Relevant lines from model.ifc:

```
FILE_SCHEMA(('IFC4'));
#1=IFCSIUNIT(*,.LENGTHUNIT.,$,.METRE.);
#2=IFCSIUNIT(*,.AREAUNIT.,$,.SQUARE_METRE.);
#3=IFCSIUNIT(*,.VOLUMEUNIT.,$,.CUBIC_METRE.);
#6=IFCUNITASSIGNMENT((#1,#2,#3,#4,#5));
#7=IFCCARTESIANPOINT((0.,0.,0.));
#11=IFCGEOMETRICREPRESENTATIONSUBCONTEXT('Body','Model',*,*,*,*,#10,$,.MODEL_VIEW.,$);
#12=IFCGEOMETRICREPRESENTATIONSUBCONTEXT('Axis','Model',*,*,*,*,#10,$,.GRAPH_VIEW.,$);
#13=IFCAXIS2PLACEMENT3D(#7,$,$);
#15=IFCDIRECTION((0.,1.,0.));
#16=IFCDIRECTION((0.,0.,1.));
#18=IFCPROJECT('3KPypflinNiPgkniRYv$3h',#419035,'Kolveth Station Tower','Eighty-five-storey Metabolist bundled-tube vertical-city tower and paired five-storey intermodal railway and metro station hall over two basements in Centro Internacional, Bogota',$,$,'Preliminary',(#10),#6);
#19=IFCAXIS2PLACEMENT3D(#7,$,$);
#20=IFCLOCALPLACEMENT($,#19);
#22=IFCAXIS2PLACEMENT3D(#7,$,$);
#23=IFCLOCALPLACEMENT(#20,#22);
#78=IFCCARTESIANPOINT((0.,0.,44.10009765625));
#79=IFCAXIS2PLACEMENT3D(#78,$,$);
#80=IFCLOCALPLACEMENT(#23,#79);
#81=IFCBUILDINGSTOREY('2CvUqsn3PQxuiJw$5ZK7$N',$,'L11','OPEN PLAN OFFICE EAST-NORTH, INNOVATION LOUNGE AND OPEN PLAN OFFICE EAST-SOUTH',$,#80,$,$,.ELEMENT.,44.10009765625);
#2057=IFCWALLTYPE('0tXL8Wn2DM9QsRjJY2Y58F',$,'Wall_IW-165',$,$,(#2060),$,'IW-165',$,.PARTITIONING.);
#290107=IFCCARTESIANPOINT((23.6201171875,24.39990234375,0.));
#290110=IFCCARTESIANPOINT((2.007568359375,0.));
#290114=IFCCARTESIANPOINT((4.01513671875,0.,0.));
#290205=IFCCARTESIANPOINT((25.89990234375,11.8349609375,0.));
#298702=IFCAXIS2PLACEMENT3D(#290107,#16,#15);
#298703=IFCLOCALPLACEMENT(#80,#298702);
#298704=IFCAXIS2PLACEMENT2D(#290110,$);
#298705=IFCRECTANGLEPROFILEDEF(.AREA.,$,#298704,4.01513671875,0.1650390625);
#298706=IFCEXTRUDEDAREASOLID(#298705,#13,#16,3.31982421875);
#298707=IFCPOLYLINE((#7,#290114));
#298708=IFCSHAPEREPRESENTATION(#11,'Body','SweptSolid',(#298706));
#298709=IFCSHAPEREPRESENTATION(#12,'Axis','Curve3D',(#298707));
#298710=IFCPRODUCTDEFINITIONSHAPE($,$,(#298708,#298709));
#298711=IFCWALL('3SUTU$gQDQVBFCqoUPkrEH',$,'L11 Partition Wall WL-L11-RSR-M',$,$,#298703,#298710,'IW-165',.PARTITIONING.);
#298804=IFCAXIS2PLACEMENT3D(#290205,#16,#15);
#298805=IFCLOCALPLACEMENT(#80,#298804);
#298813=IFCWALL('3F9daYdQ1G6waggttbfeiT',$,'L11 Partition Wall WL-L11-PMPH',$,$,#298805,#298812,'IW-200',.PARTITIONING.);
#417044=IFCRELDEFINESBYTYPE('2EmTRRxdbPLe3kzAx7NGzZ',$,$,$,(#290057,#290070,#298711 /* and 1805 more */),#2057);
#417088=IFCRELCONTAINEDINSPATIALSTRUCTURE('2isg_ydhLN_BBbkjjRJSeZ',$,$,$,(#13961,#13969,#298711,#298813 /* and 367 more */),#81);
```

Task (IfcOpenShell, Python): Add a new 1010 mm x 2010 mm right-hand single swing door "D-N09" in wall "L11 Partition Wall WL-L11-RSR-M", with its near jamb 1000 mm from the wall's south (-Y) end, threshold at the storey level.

```python
import numpy as np
import ifcopenshell
import ifcopenshell.api.feature
import ifcopenshell.api.geometry
import ifcopenshell.api.root
import ifcopenshell.api.spatial
import ifcopenshell.geom
import ifcopenshell.util.element
import ifcopenshell.util.placement
import ifcopenshell.util.representation
import ifcopenshell.util.shape
import ifcopenshell.util.unit

model = ifcopenshell.open("model.ifc")
unit_scale = ifcopenshell.util.unit.calculate_unit_scale(model)
settings = ifcopenshell.geom.settings()


def volume(element):
    """Net volume in cubic metres, openings subtracted."""
    shape = ifcopenshell.geom.create_shape(settings, element)
    return ifcopenshell.util.shape.get_volume(shape.geometry)


wall = model.by_guid("3SUTU$gQDQVBFCqoUPkrEH")
storey = ifcopenshell.util.element.get_container(wall, ifc_class="IfcBuildingStorey")
context = ifcopenshell.util.representation.get_context(model, "Model", "Body", "MODEL_VIEW")
before = volume(wall)

width, height, from_end, sill = 1.01, 2.01, 1, 0.0  # metres

# The wall runs along its own X axis, and the end named is its -X end.
wall_shape = ifcopenshell.geom.create_shape(settings, wall)
x, y, z = ifcopenshell.util.shape.get_vertices(wall_shape.geometry).T
start = x.min() + from_end
face, thickness = float(y.min()), float(y.max() - y.min())
wall_matrix = ifcopenshell.util.placement.get_local_placement(wall.ObjectPlacement)
level = ifcopenshell.util.placement.get_local_placement(storey.ObjectPlacement)[2, 3]


def in_wall(x, y):
    """Placement at x, y metres in the wall's axes, at sill height."""
    matrix = wall_matrix.copy()
    matrix[:, 3] = wall_matrix @ np.array([x / unit_scale, y / unit_scale, 0.0, 1.0])
    matrix[2, 3] = level + sill / unit_scale
    return matrix


# Opening: a box that overshoots both wall faces by 50 mm.
opening = ifcopenshell.api.root.create_entity(model, ifc_class="IfcOpeningElement", predefined_type="OPENING")
box = ifcopenshell.api.geometry.add_wall_representation(
    model, context=context, length=width, height=height, thickness=thickness + 0.1
)
ifcopenshell.api.geometry.assign_representation(model, product=opening, representation=box)
ifcopenshell.api.geometry.edit_object_placement(model, product=opening, matrix=in_wall(start, face - 0.05), is_si=False)
ifcopenshell.api.feature.add_feature(model, feature=opening, element=wall)

door = ifcopenshell.api.root.create_entity(model, ifc_class="IfcDoor", name="D-N09", predefined_type="DOOR")
door.OverallWidth, door.OverallHeight = width / unit_scale, height / unit_scale
door.OperationType = "SINGLE_SWING_RIGHT"
body = ifcopenshell.api.geometry.add_door_representation(
    model,
    context=context,
    overall_width=door.OverallWidth,
    overall_height=door.OverallHeight,
    operation_type="SINGLE_SWING_RIGHT",
    lining_properties={"LiningDepth": thickness / unit_scale, "ThresholdDepth": thickness / unit_scale},
)
ifcopenshell.api.geometry.assign_representation(model, product=door, representation=body)
ifcopenshell.api.spatial.assign_container(model, products=[door], relating_structure=storey)
ifcopenshell.api.feature.add_filling(model, opening=opening, element=door)

# The lining spans the wall, so the door starts at the wall face.
ifcopenshell.api.geometry.edit_object_placement(model, product=door, matrix=in_wall(start, face), is_si=False)

after = volume(wall)

print(f"wall volume {before:.3f} -> {after:.3f} m3")

model.write("model_updated.ifc")
```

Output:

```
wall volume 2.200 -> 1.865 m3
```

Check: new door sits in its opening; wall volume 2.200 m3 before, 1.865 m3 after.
